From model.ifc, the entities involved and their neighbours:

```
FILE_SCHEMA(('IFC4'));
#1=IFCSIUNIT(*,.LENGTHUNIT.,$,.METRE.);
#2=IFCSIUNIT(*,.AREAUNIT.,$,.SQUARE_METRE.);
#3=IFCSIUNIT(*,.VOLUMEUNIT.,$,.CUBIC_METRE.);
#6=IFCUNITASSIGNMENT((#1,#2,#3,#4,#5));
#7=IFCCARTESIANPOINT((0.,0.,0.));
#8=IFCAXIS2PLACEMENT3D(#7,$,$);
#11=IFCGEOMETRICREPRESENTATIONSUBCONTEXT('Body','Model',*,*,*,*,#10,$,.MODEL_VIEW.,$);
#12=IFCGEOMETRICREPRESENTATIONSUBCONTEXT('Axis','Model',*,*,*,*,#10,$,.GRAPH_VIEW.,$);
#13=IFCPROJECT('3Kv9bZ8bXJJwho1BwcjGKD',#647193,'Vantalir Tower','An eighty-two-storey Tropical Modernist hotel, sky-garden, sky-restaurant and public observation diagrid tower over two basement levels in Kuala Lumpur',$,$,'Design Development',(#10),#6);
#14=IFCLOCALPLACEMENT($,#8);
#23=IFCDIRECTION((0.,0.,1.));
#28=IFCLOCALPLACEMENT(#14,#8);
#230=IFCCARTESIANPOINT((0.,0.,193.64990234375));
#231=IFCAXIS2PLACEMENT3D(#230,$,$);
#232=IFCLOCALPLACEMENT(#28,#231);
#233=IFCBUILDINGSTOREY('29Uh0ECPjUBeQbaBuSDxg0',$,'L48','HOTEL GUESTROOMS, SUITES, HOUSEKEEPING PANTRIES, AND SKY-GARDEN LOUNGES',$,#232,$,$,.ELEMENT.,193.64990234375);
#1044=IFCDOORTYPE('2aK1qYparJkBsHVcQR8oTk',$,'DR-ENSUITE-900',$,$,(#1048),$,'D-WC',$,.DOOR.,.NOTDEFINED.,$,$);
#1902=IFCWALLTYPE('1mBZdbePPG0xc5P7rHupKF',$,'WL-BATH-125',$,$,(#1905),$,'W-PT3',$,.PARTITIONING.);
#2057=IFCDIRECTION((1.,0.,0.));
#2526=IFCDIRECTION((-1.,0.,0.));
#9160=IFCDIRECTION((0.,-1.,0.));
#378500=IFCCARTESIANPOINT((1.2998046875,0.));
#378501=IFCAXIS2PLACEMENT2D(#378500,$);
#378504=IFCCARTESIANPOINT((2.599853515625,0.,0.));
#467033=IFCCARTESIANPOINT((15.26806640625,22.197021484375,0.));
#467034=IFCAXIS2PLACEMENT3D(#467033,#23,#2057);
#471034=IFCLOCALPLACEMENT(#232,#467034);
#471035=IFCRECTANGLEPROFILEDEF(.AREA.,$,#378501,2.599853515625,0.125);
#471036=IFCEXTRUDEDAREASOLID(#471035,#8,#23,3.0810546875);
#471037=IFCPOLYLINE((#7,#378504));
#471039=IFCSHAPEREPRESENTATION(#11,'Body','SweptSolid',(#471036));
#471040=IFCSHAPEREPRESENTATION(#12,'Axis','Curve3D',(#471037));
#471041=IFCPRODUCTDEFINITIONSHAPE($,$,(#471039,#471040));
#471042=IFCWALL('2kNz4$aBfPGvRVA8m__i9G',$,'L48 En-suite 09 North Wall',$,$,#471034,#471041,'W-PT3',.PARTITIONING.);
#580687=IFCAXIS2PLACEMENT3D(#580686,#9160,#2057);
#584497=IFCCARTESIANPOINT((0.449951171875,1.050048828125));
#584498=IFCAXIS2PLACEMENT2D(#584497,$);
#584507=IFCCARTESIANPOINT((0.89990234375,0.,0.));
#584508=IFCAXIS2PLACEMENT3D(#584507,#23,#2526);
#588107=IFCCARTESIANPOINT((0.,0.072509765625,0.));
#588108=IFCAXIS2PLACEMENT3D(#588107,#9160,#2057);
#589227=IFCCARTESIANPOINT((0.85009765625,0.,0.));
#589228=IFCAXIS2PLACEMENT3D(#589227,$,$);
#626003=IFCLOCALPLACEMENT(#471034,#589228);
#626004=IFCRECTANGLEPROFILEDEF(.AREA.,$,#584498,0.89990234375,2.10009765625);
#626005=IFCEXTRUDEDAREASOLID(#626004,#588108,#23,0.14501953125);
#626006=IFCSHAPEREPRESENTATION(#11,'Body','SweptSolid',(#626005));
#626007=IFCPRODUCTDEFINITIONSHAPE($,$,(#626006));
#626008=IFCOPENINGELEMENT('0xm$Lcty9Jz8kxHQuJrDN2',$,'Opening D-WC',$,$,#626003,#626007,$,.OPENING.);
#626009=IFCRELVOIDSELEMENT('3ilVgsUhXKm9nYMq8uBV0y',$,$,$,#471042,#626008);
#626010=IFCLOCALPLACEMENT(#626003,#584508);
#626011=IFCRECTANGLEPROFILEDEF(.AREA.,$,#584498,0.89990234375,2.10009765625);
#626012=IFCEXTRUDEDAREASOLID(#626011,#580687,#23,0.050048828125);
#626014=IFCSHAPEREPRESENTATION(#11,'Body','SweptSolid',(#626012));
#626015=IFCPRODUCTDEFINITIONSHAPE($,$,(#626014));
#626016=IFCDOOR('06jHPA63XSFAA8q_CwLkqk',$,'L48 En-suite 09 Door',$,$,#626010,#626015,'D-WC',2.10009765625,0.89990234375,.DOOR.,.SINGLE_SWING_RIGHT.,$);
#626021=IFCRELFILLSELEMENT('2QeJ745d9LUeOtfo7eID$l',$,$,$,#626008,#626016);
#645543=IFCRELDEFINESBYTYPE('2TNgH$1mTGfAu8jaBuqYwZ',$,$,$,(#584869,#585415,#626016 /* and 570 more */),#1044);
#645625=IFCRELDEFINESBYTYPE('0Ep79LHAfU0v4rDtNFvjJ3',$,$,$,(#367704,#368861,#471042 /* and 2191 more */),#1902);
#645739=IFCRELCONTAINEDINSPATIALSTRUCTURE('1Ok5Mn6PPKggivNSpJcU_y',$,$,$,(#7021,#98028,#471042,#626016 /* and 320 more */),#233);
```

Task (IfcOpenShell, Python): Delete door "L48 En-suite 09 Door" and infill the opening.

```python
import ifcopenshell
import ifcopenshell.api.feature
import ifcopenshell.api.root
import ifcopenshell.geom
import ifcopenshell.util.shape

model = ifcopenshell.open("model.ifc")
settings = ifcopenshell.geom.settings()


def volume(element):
    """Net volume in cubic metres, openings subtracted."""
    shape = ifcopenshell.geom.create_shape(settings, element)
    return ifcopenshell.util.shape.get_volume(shape.geometry)


door = model.by_id(626016)
opening = door.FillsVoids[0].RelatingOpeningElement
wall = opening.VoidsElements[0].RelatingBuildingElement
before = volume(wall)

ifcopenshell.api.root.remove_product(model, product=door)
ifcopenshell.api.feature.remove_feature(model, feature=opening)

after = volume(wall)

print(f"wall volume {before:.3f} -> {after:.3f} m3")

model.write("model_v2.ifc")
```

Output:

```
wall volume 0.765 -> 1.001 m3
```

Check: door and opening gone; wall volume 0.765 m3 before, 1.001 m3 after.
